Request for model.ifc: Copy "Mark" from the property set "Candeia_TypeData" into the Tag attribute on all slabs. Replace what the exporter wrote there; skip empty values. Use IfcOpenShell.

First a look at what the model holds.

```python
import ifcopenshell
import ifcopenshell.util.element

model = ifcopenshell.open("model.ifc")
print(model.schema)
slabs = model.by_type("IfcSlab")
print(len(slabs), "slabs")
for e in slabs[:8]:
    source = ifcopenshell.util.element.get_pset(e, "Candeia_TypeData", "Mark")
    target = e.Tag
    print(e.id(), repr(source), repr(target), sep=" | ")
```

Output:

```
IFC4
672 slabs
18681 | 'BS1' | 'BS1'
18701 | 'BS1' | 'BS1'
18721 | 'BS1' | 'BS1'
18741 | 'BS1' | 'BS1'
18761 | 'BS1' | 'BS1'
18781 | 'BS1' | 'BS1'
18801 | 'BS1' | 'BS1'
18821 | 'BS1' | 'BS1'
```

```python
import ifcopenshell
import ifcopenshell.util.element

model = ifcopenshell.open("model.ifc")

count = 0
for e in model.by_type("IfcSlab"):
    value = ifcopenshell.util.element.get_pset(e, "Candeia_TypeData", "Mark")
    current = e.Tag
    if not value or not value.strip() or current == value:
        continue
    e.Tag = value
    count += 1

print(count, "slabs updated")

model.write("model_updated.ifc")
```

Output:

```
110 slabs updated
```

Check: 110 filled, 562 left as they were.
